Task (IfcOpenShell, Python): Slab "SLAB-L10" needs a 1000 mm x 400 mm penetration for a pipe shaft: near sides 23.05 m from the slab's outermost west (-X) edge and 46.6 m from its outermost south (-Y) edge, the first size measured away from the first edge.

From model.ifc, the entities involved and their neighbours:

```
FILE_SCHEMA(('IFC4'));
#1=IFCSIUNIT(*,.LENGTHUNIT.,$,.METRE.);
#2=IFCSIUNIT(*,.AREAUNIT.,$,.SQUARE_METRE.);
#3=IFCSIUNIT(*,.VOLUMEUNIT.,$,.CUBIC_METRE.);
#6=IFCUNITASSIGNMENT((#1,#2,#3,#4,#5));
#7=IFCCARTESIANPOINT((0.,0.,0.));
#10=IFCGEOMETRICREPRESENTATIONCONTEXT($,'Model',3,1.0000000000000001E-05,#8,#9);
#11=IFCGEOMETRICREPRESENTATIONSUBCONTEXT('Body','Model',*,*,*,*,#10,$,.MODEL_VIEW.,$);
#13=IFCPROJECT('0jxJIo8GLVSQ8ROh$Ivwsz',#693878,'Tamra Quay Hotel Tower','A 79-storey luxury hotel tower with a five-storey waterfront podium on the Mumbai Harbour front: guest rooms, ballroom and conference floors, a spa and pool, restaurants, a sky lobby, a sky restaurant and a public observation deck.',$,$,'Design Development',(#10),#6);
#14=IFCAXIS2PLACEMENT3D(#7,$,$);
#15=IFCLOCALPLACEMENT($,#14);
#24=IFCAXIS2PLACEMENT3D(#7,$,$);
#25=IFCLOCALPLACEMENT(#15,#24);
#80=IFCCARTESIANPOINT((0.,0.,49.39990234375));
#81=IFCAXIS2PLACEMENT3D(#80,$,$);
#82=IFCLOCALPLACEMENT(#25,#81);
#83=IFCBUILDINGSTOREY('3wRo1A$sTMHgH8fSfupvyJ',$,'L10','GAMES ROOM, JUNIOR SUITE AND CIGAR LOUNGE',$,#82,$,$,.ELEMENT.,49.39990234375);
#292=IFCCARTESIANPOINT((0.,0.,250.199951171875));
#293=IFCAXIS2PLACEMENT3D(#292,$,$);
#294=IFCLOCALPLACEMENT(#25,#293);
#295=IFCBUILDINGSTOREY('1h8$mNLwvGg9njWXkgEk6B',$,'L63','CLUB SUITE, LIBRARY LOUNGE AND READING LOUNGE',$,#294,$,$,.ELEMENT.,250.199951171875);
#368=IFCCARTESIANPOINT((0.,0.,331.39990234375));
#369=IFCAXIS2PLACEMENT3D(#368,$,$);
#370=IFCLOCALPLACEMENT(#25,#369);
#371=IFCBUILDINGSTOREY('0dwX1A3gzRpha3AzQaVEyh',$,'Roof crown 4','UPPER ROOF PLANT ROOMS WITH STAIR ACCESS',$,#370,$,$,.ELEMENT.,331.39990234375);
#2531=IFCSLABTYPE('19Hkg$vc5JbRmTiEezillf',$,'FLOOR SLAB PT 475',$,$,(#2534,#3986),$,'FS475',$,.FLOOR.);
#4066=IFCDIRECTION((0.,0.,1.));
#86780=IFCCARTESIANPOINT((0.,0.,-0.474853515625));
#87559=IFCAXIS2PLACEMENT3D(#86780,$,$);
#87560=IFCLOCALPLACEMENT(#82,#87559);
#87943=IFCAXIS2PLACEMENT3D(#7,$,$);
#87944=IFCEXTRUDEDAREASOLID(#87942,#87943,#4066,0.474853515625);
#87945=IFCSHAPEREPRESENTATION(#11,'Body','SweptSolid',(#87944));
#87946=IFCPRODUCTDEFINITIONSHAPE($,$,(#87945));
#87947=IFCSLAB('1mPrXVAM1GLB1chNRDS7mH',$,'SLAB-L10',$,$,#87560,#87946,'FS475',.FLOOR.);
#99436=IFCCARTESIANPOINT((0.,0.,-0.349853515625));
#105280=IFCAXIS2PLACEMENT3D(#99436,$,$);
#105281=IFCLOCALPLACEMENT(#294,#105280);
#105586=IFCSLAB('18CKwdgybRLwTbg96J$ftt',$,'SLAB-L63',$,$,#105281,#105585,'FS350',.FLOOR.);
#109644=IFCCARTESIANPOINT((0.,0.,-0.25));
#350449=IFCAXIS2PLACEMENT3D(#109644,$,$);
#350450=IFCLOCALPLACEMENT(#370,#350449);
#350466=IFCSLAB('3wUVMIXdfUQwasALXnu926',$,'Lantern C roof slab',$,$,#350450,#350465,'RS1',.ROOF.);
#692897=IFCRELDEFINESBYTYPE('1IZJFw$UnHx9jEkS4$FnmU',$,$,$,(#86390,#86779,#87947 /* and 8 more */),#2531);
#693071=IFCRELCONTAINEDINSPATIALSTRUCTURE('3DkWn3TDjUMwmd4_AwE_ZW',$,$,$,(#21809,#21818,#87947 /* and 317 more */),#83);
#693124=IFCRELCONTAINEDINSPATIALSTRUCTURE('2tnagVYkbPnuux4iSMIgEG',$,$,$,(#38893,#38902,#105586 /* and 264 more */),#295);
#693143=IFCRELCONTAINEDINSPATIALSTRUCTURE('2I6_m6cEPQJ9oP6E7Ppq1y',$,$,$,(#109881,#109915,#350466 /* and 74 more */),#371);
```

```python
import numpy as np
import ifcopenshell
import ifcopenshell.api.feature
import ifcopenshell.api.geometry
import ifcopenshell.api.root
import ifcopenshell.geom
import ifcopenshell.util.placement
import ifcopenshell.util.representation
import ifcopenshell.util.shape
import ifcopenshell.util.unit

model = ifcopenshell.open("model.ifc")
unit_scale = ifcopenshell.util.unit.calculate_unit_scale(model)
settings = ifcopenshell.geom.settings()


def volume(element):
    """Net volume in cubic metres, openings subtracted."""
    shape = ifcopenshell.geom.create_shape(settings, element)
    return ifcopenshell.util.shape.get_volume(shape.geometry)


slab = model.by_guid("1mPrXVAM1GLB1chNRDS7mH")
before = volume(slab)

# Extent in the slab's own axes, in metres. The edges named are its -X and -Y sides.
slab_shape = ifcopenshell.geom.create_shape(settings, slab)
vertices = ifcopenshell.util.shape.get_vertices(slab_shape.geometry)
x_min, y_min, bottom = vertices.min(axis=0)
top = vertices[:, 2].max()

opening = ifcopenshell.api.root.create_entity(model, ifc_class="IfcOpeningElement", name="Pipe shaft opening", predefined_type="OPENING")
context = ifcopenshell.util.representation.get_context(model, "Model", "Body", "MODEL_VIEW")
width, depth = 1, 0.4
outline = [(0.0, 0.0), (width, 0.0), (width, depth), (0.0, depth), (0.0, 0.0)]
# Overshoot both faces by 50 mm so the cut is clean.
shape = ifcopenshell.api.geometry.add_slab_representation(
    model, context=context, depth=top - bottom + 0.1, polyline=outline
)
ifcopenshell.api.geometry.assign_representation(model, product=opening, representation=shape)

matrix = ifcopenshell.util.placement.get_local_placement(slab.ObjectPlacement)
matrix[:, 3] = matrix @ np.append(np.array([x_min + 23.05, y_min + 46.6, bottom - 0.05]) / unit_scale, 1.0)
ifcopenshell.api.geometry.edit_object_placement(model, product=opening, matrix=matrix, is_si=False)
ifcopenshell.api.feature.add_feature(model, feature=opening, element=slab)

after = volume(slab)

print(f"slab volume {before:.3f} -> {after:.3f} m3")

model.write("model-out.ifc")
```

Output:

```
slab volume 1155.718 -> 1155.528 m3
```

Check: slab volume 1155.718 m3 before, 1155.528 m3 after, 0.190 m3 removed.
